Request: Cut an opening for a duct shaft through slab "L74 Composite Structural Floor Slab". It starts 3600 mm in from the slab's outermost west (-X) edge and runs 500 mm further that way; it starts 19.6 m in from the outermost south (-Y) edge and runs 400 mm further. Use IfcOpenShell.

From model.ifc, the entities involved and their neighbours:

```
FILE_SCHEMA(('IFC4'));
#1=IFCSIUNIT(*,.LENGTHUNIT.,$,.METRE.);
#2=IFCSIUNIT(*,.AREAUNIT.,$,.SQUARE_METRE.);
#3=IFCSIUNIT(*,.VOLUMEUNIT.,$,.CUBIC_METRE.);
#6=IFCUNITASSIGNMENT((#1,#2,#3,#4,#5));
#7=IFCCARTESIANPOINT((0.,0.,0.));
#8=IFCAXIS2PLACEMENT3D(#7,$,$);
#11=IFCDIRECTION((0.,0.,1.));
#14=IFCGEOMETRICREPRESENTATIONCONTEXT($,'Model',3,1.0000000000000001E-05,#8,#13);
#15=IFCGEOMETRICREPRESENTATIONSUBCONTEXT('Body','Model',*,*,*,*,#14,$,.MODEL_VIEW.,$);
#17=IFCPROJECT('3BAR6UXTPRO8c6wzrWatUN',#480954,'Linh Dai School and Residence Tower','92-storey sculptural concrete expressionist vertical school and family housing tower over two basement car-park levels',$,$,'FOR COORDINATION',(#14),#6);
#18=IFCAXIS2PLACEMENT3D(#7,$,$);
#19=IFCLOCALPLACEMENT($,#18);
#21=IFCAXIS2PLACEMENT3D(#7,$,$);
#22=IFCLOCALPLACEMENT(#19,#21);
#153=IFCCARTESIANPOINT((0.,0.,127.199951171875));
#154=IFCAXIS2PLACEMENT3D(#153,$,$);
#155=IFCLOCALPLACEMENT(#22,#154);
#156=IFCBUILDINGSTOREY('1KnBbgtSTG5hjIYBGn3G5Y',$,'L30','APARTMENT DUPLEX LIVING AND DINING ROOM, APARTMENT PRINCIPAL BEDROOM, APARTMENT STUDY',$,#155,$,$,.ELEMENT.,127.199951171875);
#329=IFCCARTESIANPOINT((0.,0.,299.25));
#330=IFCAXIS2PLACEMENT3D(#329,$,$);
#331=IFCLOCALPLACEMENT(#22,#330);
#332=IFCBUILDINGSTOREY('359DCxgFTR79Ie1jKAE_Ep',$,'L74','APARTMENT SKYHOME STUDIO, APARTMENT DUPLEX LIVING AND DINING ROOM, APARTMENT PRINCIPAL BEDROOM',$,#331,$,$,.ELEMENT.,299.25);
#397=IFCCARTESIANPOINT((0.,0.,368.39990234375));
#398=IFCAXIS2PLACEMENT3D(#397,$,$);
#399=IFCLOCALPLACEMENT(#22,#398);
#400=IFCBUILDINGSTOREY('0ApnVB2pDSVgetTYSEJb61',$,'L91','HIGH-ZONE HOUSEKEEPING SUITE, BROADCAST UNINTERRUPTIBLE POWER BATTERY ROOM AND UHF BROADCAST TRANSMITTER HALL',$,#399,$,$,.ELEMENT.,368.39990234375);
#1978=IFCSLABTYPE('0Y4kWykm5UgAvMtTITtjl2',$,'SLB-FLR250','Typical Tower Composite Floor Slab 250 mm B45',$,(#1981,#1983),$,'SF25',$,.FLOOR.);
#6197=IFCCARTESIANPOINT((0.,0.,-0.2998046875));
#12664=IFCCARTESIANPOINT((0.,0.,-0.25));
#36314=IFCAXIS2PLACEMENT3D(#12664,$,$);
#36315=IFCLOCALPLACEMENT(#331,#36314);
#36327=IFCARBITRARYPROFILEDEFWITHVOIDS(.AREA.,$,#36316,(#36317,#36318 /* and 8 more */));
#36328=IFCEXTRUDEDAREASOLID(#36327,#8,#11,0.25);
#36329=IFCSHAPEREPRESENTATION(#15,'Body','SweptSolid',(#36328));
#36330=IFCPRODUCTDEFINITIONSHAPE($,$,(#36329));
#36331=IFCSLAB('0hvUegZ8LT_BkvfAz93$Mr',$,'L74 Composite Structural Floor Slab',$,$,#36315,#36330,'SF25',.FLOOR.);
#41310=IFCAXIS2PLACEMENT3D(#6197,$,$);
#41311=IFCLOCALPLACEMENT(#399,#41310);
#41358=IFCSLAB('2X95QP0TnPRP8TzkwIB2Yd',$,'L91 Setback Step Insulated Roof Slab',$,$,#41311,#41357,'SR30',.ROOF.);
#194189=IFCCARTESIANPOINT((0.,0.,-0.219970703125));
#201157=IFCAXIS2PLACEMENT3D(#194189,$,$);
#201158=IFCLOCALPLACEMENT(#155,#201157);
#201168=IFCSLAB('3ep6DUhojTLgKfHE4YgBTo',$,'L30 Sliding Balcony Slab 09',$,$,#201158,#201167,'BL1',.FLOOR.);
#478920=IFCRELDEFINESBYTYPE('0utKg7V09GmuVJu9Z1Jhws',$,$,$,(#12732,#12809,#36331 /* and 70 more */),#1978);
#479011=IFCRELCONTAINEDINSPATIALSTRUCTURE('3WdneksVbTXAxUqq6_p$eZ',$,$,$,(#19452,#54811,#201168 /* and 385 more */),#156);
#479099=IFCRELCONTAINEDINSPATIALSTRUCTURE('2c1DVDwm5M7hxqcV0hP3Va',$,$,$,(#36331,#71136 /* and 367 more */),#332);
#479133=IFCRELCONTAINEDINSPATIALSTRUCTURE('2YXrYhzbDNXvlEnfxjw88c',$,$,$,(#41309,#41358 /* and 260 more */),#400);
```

```python
import numpy as np
import ifcopenshell
import ifcopenshell.api.feature
import ifcopenshell.api.geometry
import ifcopenshell.api.root
import ifcopenshell.geom
import ifcopenshell.util.placement
import ifcopenshell.util.representation
import ifcopenshell.util.shape
import ifcopenshell.util.unit

model = ifcopenshell.open("model.ifc")
unit_scale = ifcopenshell.util.unit.calculate_unit_scale(model)
settings = ifcopenshell.geom.settings()


def volume(element):
    """Net volume in cubic metres, openings subtracted."""
    shape = ifcopenshell.geom.create_shape(settings, element)
    return ifcopenshell.util.shape.get_volume(shape.geometry)


slab = model.by_guid("0hvUegZ8LT_BkvfAz93$Mr")
before = volume(slab)

# Extent in the slab's own axes, in metres. The edges named are its -X and -Y sides.
slab_shape = ifcopenshell.geom.create_shape(settings, slab)
vertices = ifcopenshell.util.shape.get_vertices(slab_shape.geometry)
x_min, y_min, bottom = vertices.min(axis=0)
top = vertices[:, 2].max()

opening = ifcopenshell.api.root.create_entity(model, ifc_class="IfcOpeningElement", name="Duct shaft opening", predefined_type="OPENING")
context = ifcopenshell.util.representation.get_context(model, "Model", "Body", "MODEL_VIEW")
width, depth = 0.5, 0.4
outline = [(0.0, 0.0), (width, 0.0), (width, depth), (0.0, depth), (0.0, 0.0)]
# Overshoot both faces by 50 mm so the cut is clean.
shape = ifcopenshell.api.geometry.add_slab_representation(
    model, context=context, depth=top - bottom + 0.1, polyline=outline
)
ifcopenshell.api.geometry.assign_representation(model, product=opening, representation=shape)

matrix = ifcopenshell.util.placement.get_local_placement(slab.ObjectPlacement)
matrix[:, 3] = matrix @ np.append(np.array([x_min + 3.6, y_min + 19.6, bottom - 0.05]) / unit_scale, 1.0)
ifcopenshell.api.geometry.edit_object_placement(model, product=opening, matrix=matrix, is_si=False)
ifcopenshell.api.feature.add_feature(model, feature=opening, element=slab)

after = volume(slab)

print(f"slab volume {before:.3f} -> {after:.3f} m3")

model.write("model_v2.ifc")
```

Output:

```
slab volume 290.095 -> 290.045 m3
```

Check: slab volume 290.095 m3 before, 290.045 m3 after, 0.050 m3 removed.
